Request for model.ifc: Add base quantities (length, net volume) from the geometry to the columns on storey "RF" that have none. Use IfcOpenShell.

First a look at what the model holds.

```python
import ifcopenshell
import ifcopenshell.util.element
import ifcopenshell.util.unit

model = ifcopenshell.open("model.ifc")
print(model.schema)
for unit_type in ("LENGTHUNIT", "AREAUNIT", "VOLUMEUNIT"):
    print(unit_type, ifcopenshell.util.unit.calculate_unit_scale(model, unit_type))
storey = next(s for s in model.by_type("IfcBuildingStorey") if s.Name == "RF")
columns = [e for e in ifcopenshell.util.element.get_decomposition(storey) if e.is_a("IfcColumn")]
for e in sorted(columns, key=lambda e: e.id()):
    print(e.id(), e.is_a(), e.Name, list(ifcopenshell.util.element.get_psets(e, qtos_only=True)), sep=" | ")
```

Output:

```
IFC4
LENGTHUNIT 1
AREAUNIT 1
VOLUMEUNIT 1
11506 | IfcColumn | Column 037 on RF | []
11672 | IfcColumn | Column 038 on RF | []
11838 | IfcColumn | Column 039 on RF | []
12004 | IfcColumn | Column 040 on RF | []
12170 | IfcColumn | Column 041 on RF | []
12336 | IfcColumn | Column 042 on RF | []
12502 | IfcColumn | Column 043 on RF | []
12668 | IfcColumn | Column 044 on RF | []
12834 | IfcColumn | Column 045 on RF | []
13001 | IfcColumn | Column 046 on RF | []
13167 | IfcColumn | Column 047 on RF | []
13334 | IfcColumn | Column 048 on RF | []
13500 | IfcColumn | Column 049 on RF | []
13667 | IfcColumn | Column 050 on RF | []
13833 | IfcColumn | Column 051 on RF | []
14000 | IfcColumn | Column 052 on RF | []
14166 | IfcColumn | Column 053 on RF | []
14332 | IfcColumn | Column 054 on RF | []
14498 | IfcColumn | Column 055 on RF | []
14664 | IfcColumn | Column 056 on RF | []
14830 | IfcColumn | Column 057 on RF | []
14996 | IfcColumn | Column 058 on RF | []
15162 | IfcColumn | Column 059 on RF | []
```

```python
import ifcopenshell
import ifcopenshell.api.pset
import ifcopenshell.geom
import ifcopenshell.util.element
import ifcopenshell.util.shape
import ifcopenshell.util.unit

model = ifcopenshell.open("model.ifc")
unit_scale = ifcopenshell.util.unit.calculate_unit_scale(model)
volume_scale = ifcopenshell.util.unit.calculate_unit_scale(model, "VOLUMEUNIT")
settings = ifcopenshell.geom.settings()

storey = next(s for s in model.by_type("IfcBuildingStorey") if s.Name == "RF")
columns = [e for e in ifcopenshell.util.element.get_decomposition(storey) if e.is_a("IfcColumn")]

for e in sorted(columns, key=lambda e: e.id()):
    if ifcopenshell.util.element.get_psets(e, qtos_only=True, should_inherit=False):
        continue
    # Geometry comes back in metres, in the element's own axes.
    shape = ifcopenshell.geom.create_shape(settings, e)
    values = {
        "Length": ifcopenshell.util.shape.get_z(shape.geometry) / unit_scale,
        "NetVolume": ifcopenshell.util.shape.get_volume(shape.geometry) / volume_scale,
    }
    qto = ifcopenshell.api.pset.add_qto(model, product=e, name="Qto_ColumnBaseQuantities")
    ifcopenshell.api.pset.edit_qto(model, qto=qto, properties=values)
    print(e.id(), {k: round(v, 3) for k, v in values.items()})

model.write("model_updated.ifc")
```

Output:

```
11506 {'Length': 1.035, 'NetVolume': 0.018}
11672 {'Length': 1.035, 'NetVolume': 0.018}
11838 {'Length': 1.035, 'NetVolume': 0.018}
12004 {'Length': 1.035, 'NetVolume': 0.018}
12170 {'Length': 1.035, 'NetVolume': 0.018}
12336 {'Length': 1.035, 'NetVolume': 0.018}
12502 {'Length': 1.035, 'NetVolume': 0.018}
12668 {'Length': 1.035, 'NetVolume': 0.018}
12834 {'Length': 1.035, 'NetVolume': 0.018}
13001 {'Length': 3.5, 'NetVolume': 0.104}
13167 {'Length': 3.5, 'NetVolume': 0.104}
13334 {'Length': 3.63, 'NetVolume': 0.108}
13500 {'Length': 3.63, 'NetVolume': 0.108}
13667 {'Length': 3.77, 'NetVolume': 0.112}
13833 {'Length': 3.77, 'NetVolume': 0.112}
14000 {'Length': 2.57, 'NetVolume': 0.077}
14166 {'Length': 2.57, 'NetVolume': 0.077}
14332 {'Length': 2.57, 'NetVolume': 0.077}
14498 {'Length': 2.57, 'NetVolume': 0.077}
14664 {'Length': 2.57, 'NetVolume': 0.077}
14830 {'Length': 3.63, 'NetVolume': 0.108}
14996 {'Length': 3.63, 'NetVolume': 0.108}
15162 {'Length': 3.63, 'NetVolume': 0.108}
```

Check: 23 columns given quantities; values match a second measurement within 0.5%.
